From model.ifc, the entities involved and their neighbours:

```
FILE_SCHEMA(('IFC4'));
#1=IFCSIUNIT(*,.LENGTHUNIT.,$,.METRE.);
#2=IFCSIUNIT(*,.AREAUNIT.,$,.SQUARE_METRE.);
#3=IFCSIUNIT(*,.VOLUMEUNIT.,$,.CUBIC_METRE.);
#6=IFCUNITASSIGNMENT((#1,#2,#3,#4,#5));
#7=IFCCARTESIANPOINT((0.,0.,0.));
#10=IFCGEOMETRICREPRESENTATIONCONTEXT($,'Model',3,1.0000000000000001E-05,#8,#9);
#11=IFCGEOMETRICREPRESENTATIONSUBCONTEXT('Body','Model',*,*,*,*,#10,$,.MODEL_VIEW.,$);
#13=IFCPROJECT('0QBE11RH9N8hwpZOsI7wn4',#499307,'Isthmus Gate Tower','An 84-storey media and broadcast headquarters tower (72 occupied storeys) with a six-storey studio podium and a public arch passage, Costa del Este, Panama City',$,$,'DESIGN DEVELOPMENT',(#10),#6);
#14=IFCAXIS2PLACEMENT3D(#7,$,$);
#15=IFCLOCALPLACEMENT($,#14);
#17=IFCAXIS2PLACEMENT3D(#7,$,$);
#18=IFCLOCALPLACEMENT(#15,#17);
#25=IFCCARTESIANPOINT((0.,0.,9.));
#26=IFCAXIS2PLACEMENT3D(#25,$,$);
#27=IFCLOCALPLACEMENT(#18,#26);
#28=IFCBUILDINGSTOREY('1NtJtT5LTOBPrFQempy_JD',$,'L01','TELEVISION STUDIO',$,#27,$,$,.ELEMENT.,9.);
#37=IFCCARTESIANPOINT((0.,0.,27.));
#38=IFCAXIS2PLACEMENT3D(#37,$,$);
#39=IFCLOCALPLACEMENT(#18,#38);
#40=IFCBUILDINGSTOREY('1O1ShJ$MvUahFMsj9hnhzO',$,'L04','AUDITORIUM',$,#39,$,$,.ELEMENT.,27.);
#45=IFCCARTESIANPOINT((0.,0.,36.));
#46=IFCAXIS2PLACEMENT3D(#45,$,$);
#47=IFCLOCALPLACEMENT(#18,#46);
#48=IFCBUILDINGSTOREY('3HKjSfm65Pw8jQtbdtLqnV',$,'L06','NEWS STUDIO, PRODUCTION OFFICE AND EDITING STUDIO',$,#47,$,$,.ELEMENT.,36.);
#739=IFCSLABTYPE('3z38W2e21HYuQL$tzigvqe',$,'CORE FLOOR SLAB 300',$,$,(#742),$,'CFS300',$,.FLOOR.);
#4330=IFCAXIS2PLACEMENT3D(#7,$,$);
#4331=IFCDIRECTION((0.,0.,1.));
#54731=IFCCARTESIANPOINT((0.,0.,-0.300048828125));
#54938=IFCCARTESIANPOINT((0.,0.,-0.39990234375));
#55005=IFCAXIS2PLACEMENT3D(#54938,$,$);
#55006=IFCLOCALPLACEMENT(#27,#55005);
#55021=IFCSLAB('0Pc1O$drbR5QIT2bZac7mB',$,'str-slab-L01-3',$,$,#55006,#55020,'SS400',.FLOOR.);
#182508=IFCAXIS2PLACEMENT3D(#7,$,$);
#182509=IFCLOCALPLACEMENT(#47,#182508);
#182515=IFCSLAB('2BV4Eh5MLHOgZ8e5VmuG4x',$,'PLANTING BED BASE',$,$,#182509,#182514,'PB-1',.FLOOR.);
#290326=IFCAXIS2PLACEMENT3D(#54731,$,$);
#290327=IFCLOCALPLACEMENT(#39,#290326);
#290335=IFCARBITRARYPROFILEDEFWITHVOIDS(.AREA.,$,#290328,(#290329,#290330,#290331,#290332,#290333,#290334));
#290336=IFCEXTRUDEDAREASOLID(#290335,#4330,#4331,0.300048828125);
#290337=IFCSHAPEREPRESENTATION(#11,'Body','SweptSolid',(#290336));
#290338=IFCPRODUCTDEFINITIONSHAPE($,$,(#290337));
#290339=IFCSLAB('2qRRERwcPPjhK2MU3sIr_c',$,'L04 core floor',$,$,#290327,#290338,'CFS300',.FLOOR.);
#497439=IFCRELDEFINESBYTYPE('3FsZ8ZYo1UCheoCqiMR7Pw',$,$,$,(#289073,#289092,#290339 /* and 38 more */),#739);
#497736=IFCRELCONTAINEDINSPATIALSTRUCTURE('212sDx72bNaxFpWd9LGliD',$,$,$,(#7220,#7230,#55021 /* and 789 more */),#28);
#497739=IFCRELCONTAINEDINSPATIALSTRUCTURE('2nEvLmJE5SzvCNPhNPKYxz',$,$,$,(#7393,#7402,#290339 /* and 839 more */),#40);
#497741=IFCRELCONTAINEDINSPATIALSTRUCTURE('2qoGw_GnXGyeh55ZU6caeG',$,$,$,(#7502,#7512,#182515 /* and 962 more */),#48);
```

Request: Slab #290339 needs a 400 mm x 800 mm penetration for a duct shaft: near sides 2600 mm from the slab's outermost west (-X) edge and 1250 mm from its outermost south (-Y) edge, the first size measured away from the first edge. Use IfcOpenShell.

```python
import numpy as np
import ifcopenshell
import ifcopenshell.api.feature
import ifcopenshell.api.geometry
import ifcopenshell.api.root
import ifcopenshell.geom
import ifcopenshell.util.placement
import ifcopenshell.util.representation
import ifcopenshell.util.shape
import ifcopenshell.util.unit

model = ifcopenshell.open("model.ifc")
unit_scale = ifcopenshell.util.unit.calculate_unit_scale(model)
settings = ifcopenshell.geom.settings()


def volume(element):
    """Net volume in cubic metres, openings subtracted."""
    shape = ifcopenshell.geom.create_shape(settings, element)
    return ifcopenshell.util.shape.get_volume(shape.geometry)


slab = model.by_guid("2qRRERwcPPjhK2MU3sIr_c")
before = volume(slab)

# Extent in the slab's own axes, in metres. The edges named are its -X and -Y sides.
slab_shape = ifcopenshell.geom.create_shape(settings, slab)
vertices = ifcopenshell.util.shape.get_vertices(slab_shape.geometry)
x_min, y_min, bottom = vertices.min(axis=0)
top = vertices[:, 2].max()

opening = ifcopenshell.api.root.create_entity(model, ifc_class="IfcOpeningElement", name="Duct shaft opening", predefined_type="OPENING")
context = ifcopenshell.util.representation.get_context(model, "Model", "Body", "MODEL_VIEW")
width, depth = 0.4, 0.8
outline = [(0.0, 0.0), (width, 0.0), (width, depth), (0.0, depth), (0.0, 0.0)]
# Overshoot both faces by 50 mm so the cut is clean.
shape = ifcopenshell.api.geometry.add_slab_representation(
    model, context=context, depth=top - bottom + 0.1, polyline=outline
)
ifcopenshell.api.geometry.assign_representation(model, product=opening, representation=shape)

matrix = ifcopenshell.util.placement.get_local_placement(slab.ObjectPlacement)
matrix[:, 3] = matrix @ np.append(np.array([x_min + 2.6, y_min + 1.25, bottom - 0.05]) / unit_scale, 1.0)
ifcopenshell.api.geometry.edit_object_placement(model, product=opening, matrix=matrix, is_si=False)
ifcopenshell.api.feature.add_feature(model, feature=opening, element=slab)

after = volume(slab)

print(f"slab volume {before:.3f} -> {after:.3f} m3")

model.write("model_edited.ifc")
```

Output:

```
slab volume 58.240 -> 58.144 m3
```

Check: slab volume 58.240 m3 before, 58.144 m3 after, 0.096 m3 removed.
